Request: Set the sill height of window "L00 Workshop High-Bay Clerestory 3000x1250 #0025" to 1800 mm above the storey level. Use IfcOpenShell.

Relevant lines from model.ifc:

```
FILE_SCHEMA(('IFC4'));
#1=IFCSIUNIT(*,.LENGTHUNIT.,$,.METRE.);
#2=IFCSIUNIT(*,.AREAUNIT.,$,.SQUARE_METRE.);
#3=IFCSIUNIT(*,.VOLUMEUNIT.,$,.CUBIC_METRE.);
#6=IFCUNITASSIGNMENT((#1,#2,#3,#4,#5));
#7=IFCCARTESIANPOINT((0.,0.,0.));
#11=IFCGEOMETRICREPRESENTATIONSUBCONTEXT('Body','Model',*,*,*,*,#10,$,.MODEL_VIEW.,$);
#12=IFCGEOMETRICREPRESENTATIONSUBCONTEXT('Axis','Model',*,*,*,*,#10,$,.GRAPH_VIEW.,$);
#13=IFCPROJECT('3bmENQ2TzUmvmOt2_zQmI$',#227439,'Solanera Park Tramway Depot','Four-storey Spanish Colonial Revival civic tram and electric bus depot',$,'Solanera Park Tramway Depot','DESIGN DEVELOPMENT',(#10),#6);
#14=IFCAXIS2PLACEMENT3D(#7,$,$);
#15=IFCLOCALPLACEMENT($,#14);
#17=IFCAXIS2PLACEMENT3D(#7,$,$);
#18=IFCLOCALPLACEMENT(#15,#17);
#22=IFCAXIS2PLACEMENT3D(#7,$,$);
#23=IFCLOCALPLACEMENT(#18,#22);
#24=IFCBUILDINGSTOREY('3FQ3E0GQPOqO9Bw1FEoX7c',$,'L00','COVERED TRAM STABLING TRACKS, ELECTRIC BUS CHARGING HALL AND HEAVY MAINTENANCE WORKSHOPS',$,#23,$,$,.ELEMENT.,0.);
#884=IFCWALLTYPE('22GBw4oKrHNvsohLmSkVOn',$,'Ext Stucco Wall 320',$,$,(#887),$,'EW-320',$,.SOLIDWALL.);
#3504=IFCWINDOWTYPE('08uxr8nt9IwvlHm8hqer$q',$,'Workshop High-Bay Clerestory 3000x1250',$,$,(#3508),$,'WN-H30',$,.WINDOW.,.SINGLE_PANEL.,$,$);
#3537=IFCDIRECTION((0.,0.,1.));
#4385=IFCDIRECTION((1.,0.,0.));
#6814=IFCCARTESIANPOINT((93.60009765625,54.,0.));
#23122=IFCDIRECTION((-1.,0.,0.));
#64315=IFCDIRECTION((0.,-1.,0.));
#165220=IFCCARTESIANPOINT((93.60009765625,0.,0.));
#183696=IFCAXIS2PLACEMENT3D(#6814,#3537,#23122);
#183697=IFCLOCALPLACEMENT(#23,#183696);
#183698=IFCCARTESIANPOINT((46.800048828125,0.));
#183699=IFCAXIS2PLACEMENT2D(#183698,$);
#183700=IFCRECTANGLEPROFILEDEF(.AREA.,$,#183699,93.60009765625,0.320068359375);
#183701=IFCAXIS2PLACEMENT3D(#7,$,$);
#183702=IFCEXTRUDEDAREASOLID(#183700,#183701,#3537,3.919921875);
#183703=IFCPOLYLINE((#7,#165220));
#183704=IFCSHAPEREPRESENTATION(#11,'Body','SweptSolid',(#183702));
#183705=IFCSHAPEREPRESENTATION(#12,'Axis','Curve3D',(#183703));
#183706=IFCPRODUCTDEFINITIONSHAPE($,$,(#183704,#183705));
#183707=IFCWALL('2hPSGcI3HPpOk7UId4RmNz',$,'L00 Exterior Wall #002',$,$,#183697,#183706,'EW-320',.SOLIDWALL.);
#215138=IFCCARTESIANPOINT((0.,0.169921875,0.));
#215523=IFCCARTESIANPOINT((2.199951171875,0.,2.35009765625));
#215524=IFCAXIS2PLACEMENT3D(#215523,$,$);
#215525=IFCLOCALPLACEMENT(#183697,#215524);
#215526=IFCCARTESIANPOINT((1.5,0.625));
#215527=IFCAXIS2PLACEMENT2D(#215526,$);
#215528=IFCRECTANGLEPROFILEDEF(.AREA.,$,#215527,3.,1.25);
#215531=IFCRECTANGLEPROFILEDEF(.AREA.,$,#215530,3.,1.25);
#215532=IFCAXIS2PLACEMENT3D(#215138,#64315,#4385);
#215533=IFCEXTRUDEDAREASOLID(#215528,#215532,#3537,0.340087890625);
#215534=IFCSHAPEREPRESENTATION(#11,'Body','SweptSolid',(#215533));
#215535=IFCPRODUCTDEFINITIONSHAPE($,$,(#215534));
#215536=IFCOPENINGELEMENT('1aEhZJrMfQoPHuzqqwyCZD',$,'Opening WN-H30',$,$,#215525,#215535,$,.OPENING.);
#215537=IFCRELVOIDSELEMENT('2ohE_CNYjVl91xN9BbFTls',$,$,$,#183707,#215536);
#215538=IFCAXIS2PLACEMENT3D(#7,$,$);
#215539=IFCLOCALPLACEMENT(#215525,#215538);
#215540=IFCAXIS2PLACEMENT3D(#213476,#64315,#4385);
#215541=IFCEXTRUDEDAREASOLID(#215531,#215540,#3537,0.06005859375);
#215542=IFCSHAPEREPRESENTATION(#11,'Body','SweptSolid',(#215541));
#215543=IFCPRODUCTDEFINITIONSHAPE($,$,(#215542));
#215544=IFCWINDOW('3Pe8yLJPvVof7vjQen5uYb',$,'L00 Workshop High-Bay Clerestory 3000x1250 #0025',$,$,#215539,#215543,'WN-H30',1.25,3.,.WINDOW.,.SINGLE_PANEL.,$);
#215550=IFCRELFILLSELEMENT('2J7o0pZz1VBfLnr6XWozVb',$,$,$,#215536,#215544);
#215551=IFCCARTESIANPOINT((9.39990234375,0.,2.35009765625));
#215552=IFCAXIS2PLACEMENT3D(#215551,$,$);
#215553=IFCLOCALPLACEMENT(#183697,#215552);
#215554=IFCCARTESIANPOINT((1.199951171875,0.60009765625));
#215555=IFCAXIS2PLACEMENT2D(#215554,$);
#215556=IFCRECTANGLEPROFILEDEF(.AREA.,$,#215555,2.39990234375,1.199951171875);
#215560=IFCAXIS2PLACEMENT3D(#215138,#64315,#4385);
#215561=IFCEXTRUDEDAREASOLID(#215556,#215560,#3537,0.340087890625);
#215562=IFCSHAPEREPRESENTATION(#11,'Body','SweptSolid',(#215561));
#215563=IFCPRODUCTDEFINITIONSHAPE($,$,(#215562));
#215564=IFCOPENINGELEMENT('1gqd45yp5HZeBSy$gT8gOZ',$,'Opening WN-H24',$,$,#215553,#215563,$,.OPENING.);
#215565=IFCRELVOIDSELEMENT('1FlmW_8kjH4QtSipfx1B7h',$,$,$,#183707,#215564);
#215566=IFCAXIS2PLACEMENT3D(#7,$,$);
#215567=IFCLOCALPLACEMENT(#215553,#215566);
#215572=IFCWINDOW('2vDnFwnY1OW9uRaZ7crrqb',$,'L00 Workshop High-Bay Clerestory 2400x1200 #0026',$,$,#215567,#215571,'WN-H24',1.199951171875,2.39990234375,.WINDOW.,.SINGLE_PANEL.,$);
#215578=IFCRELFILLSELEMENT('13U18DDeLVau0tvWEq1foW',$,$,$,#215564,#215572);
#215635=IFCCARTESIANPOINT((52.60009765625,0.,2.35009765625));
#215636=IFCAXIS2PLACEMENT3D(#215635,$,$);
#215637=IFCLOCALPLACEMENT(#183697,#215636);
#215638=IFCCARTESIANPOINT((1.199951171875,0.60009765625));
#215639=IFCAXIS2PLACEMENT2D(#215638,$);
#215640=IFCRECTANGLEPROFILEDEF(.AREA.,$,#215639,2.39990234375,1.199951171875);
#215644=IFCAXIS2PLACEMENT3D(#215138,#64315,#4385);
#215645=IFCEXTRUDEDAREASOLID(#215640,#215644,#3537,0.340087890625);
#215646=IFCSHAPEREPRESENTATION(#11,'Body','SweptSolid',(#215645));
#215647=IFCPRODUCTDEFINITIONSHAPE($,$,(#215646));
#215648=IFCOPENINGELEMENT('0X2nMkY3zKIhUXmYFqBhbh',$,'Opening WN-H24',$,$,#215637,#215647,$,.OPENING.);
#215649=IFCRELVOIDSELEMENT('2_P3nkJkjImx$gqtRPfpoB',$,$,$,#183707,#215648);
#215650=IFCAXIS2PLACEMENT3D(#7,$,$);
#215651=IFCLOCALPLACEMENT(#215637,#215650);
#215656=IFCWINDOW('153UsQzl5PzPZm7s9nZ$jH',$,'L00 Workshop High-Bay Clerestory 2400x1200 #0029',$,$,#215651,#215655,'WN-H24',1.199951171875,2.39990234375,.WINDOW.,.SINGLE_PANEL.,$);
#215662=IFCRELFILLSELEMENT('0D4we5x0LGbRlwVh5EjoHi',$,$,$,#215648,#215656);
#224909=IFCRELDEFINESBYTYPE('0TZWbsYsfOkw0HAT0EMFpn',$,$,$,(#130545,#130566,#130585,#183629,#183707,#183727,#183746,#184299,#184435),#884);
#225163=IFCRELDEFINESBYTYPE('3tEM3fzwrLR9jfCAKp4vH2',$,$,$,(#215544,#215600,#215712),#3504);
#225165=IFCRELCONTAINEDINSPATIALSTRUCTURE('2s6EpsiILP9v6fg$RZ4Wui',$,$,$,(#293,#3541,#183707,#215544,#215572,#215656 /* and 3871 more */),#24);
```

```python
import numpy as np
import ifcopenshell
import ifcopenshell.api.geometry
import ifcopenshell.geom
import ifcopenshell.util.element
import ifcopenshell.util.placement
import ifcopenshell.util.shape
import ifcopenshell.util.unit

model = ifcopenshell.open("model.ifc")
unit_scale = ifcopenshell.util.unit.calculate_unit_scale(model)

window = model.by_guid("3Pe8yLJPvVof7vjQen5uYb")
opening = window.FillsVoids[0].RelatingOpeningElement
storey = ifcopenshell.util.element.get_container(window, ifc_class="IfcBuildingStorey")
level = ifcopenshell.util.placement.get_local_placement(storey.ObjectPlacement)[2, 3]

# The opening's origin need not be at the sill, so measure its lowest point.
shape = ifcopenshell.geom.create_shape(ifcopenshell.geom.settings(), opening)
bottom = ifcopenshell.util.shape.get_shape_bottom_elevation(shape, shape.geometry) / unit_scale
dz = level + 1.8 / unit_scale - bottom

shift = np.array([0.0, 0.0, dz])
# The window is placed relative to its opening, so it follows when the opening moves.
matrix = ifcopenshell.util.placement.get_local_placement(opening.ObjectPlacement)
matrix[:3, 3] += shift
ifcopenshell.api.geometry.edit_object_placement(
    model, product=opening, matrix=matrix, is_si=False, should_transform_children=True
)

print(f"moved by {dz * unit_scale:+.3f} m")

model.write("model_v2.ifc")
```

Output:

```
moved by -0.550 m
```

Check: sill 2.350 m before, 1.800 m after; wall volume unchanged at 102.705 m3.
